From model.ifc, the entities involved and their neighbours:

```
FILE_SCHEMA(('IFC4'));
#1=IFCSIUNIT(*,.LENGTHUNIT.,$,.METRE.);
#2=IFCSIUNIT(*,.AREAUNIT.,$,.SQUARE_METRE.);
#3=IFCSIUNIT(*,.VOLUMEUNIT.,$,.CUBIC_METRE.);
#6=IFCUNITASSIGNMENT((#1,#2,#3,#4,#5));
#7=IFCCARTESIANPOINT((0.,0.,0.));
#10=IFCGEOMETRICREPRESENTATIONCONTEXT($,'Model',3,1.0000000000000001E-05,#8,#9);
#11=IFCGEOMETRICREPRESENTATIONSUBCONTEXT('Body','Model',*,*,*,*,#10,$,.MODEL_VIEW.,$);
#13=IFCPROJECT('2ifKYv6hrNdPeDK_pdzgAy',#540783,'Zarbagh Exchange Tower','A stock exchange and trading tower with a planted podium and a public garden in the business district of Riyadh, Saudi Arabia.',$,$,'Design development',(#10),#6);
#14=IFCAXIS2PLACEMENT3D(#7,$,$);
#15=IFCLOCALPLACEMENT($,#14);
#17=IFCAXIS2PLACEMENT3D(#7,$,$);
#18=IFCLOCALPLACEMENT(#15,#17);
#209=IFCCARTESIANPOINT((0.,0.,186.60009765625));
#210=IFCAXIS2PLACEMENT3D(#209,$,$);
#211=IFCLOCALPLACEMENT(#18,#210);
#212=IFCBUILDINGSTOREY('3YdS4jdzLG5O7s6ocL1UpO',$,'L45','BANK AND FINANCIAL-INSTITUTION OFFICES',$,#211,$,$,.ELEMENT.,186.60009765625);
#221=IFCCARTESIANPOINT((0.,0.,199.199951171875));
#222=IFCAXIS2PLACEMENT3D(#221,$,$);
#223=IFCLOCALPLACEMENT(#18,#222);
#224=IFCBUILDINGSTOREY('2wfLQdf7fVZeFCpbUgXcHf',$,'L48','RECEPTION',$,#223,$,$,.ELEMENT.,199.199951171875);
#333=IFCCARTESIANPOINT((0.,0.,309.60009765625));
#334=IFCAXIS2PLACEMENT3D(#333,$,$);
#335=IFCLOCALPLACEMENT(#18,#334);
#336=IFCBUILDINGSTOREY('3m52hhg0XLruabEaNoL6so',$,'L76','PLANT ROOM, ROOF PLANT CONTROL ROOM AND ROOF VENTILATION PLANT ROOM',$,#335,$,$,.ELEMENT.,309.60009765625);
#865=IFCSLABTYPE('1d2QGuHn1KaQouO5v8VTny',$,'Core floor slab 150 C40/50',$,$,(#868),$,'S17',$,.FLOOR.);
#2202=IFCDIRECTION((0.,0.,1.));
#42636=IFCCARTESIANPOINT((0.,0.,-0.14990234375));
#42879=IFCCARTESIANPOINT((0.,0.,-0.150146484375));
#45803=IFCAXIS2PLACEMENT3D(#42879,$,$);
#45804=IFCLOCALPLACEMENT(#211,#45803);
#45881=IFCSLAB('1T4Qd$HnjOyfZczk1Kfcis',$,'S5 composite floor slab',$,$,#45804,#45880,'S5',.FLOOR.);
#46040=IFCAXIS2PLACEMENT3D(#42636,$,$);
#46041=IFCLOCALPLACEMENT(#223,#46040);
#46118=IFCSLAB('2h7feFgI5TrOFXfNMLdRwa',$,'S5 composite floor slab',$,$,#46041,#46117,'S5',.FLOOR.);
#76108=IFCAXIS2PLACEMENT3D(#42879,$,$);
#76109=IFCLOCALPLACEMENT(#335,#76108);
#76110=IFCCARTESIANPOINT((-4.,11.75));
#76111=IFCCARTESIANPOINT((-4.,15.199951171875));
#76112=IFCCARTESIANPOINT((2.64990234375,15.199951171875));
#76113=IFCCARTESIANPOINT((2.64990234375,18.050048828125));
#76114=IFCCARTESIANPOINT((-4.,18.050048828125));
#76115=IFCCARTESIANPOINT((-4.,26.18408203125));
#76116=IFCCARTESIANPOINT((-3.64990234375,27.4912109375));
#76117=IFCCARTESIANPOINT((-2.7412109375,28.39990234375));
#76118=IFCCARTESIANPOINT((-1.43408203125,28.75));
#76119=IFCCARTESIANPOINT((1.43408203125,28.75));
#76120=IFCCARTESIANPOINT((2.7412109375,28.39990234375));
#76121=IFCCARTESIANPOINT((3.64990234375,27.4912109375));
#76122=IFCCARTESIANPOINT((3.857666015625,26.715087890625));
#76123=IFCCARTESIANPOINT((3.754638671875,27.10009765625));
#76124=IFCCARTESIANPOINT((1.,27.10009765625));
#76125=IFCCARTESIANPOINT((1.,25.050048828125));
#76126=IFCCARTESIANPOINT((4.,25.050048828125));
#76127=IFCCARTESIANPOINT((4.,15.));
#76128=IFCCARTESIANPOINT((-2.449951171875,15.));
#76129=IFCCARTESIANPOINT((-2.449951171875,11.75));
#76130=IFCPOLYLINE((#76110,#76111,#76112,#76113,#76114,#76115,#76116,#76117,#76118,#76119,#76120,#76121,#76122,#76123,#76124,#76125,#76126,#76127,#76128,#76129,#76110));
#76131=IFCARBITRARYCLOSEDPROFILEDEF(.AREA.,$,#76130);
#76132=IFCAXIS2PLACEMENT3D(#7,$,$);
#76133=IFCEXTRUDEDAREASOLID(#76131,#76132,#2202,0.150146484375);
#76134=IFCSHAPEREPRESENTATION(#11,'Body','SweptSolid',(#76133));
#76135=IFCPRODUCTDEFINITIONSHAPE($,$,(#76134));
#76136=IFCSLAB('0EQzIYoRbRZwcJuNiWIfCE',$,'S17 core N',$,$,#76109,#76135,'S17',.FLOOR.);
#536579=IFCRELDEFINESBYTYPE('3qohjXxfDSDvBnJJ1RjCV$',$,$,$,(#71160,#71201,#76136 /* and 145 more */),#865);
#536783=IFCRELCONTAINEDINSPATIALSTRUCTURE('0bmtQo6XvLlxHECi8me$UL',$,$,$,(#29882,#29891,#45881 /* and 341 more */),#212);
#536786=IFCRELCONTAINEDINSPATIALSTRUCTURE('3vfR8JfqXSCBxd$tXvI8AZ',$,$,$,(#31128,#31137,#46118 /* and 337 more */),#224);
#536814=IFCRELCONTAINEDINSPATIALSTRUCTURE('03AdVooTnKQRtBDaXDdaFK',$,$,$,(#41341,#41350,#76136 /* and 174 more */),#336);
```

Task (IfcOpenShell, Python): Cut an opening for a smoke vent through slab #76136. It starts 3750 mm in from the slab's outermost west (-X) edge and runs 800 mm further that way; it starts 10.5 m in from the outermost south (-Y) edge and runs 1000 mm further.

```python
import numpy as np
import ifcopenshell
import ifcopenshell.api.feature
import ifcopenshell.api.geometry
import ifcopenshell.api.root
import ifcopenshell.geom
import ifcopenshell.util.placement
import ifcopenshell.util.representation
import ifcopenshell.util.shape
import ifcopenshell.util.unit

model = ifcopenshell.open("model.ifc")
unit_scale = ifcopenshell.util.unit.calculate_unit_scale(model)
settings = ifcopenshell.geom.settings()


def volume(element):
    """Net volume in cubic metres, openings subtracted."""
    shape = ifcopenshell.geom.create_shape(settings, element)
    return ifcopenshell.util.shape.get_volume(shape.geometry)


slab = model.by_id(76136)
before = volume(slab)

# Extent in the slab's own axes, in metres. The edges named are its -X and -Y sides.
slab_shape = ifcopenshell.geom.create_shape(settings, slab)
vertices = ifcopenshell.util.shape.get_vertices(slab_shape.geometry)
x_min, y_min, bottom = vertices.min(axis=0)
top = vertices[:, 2].max()

opening = ifcopenshell.api.root.create_entity(model, ifc_class="IfcOpeningElement", name="Smoke vent opening", predefined_type="OPENING")
context = ifcopenshell.util.representation.get_context(model, "Model", "Body", "MODEL_VIEW")
width, depth = 0.8, 1
outline = [(0.0, 0.0), (width, 0.0), (width, depth), (0.0, depth), (0.0, 0.0)]
# Overshoot both faces by 50 mm so the cut is clean.
shape = ifcopenshell.api.geometry.add_slab_representation(
    model, context=context, depth=top - bottom + 0.1, polyline=outline
)
ifcopenshell.api.geometry.assign_representation(model, product=opening, representation=shape)

matrix = ifcopenshell.util.placement.get_local_placement(slab.ObjectPlacement)
matrix[:, 3] = matrix @ np.append(np.array([x_min + 3.75, y_min + 10.5, bottom - 0.05]) / unit_scale, 1.0)
ifcopenshell.api.geometry.edit_object_placement(model, product=opening, matrix=matrix, is_si=False)
ifcopenshell.api.feature.add_feature(model, feature=opening, element=slab)

after = volume(slab)

print(f"slab volume {before:.3f} -> {after:.3f} m3")

model.write("model_updated.ifc")
```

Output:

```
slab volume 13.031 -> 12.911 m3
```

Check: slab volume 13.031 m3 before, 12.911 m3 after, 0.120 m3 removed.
